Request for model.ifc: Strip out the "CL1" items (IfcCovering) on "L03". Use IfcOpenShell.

First a look at what the model holds.

```python
import ifcopenshell
import ifcopenshell.util.element

model = ifcopenshell.open("model.ifc")
print(model.schema)
storey = next(s for s in model.by_type("IfcBuildingStorey") if s.Name == "L03")
coverings = [e for e in ifcopenshell.util.element.get_decomposition(storey) if e.is_a("IfcCovering")]
seen = {}
for e in coverings:
    element_type = ifcopenshell.util.element.get_type(e)
    name = element_type.Name if element_type not in (None, e) else None
    seen[name] = seen.get(name, 0) + 1
for name, count in sorted(seen.items(), key=str):
    print(count, "x", name)
```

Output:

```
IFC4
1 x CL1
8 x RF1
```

```python
import ifcopenshell
import ifcopenshell.api.root
import ifcopenshell.util.element

model = ifcopenshell.open("model.ifc")

storey = next(s for s in model.by_type("IfcBuildingStorey") if s.Name == "L03")
coverings = [e for e in ifcopenshell.util.element.get_decomposition(storey) if e.is_a("IfcCovering")]
targets = [e for e in coverings if (t := ifcopenshell.util.element.get_type(e)) not in (None, e) and t.Name == "CL1"]

for e in targets:
    ifcopenshell.api.root.remove_product(model, product=e)
print(len(targets), "removed")

model.write("model_updated.ifc")
```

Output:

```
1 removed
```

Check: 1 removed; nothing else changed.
